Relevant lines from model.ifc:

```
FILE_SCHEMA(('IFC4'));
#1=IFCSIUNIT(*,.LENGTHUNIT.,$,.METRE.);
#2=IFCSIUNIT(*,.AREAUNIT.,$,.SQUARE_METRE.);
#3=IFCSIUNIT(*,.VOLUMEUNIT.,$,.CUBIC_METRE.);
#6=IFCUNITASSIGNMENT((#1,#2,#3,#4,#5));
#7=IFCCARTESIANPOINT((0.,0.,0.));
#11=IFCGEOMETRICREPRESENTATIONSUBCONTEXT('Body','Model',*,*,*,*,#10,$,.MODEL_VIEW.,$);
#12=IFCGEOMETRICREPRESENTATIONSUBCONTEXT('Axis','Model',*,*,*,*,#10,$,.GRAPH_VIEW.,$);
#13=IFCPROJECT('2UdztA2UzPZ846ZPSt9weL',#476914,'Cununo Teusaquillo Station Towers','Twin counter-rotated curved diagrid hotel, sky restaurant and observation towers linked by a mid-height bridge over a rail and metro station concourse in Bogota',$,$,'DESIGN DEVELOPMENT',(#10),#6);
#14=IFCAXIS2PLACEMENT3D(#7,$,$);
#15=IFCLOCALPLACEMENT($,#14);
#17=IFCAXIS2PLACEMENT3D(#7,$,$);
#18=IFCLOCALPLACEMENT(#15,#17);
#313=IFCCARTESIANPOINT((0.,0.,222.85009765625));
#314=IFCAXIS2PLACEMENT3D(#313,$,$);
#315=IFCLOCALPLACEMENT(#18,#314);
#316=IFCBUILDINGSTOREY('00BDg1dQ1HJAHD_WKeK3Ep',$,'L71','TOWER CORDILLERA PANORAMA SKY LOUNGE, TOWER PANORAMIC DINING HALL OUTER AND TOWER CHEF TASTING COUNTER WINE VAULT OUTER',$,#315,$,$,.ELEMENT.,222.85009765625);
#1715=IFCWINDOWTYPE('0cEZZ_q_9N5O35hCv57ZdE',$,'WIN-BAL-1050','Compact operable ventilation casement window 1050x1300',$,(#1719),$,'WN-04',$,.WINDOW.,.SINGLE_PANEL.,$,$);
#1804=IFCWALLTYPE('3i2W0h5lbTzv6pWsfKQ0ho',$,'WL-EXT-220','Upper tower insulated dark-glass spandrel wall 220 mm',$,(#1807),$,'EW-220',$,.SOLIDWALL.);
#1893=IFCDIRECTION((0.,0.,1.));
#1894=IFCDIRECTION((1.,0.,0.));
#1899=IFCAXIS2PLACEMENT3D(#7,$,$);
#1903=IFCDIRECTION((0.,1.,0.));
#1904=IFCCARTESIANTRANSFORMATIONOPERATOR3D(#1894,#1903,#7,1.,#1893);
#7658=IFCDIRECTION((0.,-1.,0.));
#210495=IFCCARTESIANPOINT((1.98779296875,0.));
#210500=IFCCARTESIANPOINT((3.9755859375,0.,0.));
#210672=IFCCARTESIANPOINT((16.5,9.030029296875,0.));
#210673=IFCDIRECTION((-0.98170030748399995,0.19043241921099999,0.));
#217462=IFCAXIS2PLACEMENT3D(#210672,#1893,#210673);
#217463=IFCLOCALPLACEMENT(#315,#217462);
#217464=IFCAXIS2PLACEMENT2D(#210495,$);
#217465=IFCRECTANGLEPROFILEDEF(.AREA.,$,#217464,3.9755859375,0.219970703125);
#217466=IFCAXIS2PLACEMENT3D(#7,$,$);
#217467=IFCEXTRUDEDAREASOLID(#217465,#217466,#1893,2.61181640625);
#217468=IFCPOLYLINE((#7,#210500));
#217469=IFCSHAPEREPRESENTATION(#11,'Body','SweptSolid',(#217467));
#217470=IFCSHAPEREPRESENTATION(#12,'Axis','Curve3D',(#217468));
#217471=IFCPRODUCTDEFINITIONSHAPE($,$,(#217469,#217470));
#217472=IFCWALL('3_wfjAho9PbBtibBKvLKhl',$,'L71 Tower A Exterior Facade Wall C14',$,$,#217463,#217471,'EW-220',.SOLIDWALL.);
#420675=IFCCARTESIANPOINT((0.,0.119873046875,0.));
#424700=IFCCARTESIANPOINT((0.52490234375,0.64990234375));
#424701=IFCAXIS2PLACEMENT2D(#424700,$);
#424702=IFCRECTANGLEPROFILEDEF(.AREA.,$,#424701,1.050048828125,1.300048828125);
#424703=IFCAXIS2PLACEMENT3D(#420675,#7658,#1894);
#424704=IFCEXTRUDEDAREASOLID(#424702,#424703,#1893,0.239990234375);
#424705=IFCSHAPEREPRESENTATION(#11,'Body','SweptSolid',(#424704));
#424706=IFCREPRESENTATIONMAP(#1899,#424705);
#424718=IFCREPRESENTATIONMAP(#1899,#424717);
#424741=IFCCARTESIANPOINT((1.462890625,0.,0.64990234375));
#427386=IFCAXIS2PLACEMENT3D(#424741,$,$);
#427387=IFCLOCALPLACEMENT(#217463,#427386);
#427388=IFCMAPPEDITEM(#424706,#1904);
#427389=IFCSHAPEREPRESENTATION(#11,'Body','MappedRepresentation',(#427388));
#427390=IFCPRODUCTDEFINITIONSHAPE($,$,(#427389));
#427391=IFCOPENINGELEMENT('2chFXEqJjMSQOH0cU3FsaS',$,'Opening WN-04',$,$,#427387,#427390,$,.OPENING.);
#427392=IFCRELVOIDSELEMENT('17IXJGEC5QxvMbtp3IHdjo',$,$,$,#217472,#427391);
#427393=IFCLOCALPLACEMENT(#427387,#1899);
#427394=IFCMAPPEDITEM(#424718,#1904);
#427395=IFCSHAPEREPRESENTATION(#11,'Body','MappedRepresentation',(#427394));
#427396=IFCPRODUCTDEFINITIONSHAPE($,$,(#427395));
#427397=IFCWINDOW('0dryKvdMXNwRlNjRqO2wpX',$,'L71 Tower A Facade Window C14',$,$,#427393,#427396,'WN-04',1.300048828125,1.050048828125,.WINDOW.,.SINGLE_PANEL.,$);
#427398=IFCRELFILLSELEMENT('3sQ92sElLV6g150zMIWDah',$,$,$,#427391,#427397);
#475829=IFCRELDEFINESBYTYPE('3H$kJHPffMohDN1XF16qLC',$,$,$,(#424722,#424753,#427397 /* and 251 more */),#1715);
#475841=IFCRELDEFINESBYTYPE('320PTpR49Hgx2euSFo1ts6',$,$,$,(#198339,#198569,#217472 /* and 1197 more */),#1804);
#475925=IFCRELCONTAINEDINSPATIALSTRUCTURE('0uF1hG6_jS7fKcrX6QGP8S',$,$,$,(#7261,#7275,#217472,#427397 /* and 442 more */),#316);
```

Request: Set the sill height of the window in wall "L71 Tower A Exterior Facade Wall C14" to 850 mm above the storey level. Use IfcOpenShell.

```python
import numpy as np
import ifcopenshell
import ifcopenshell.api.geometry
import ifcopenshell.geom
import ifcopenshell.util.element
import ifcopenshell.util.placement
import ifcopenshell.util.shape
import ifcopenshell.util.unit

model = ifcopenshell.open("model.ifc")
unit_scale = ifcopenshell.util.unit.calculate_unit_scale(model)

window = model.by_guid("0dryKvdMXNwRlNjRqO2wpX")
opening = window.FillsVoids[0].RelatingOpeningElement
storey = ifcopenshell.util.element.get_container(window, ifc_class="IfcBuildingStorey")
level = ifcopenshell.util.placement.get_local_placement(storey.ObjectPlacement)[2, 3]

# The opening's origin need not be at the sill, so measure its lowest point.
shape = ifcopenshell.geom.create_shape(ifcopenshell.geom.settings(), opening)
bottom = ifcopenshell.util.shape.get_shape_bottom_elevation(shape, shape.geometry) / unit_scale
dz = level + 0.85 / unit_scale - bottom

shift = np.array([0.0, 0.0, dz])
# The window is placed relative to its opening, so it follows when the opening moves.
matrix = ifcopenshell.util.placement.get_local_placement(opening.ObjectPlacement)
matrix[:3, 3] += shift
ifcopenshell.api.geometry.edit_object_placement(
    model, product=opening, matrix=matrix, is_si=False, should_transform_children=True
)

print(f"moved by {dz * unit_scale:+.3f} m")

model.write("model_v2.ifc")
```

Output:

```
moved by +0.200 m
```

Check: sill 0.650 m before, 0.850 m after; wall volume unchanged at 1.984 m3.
